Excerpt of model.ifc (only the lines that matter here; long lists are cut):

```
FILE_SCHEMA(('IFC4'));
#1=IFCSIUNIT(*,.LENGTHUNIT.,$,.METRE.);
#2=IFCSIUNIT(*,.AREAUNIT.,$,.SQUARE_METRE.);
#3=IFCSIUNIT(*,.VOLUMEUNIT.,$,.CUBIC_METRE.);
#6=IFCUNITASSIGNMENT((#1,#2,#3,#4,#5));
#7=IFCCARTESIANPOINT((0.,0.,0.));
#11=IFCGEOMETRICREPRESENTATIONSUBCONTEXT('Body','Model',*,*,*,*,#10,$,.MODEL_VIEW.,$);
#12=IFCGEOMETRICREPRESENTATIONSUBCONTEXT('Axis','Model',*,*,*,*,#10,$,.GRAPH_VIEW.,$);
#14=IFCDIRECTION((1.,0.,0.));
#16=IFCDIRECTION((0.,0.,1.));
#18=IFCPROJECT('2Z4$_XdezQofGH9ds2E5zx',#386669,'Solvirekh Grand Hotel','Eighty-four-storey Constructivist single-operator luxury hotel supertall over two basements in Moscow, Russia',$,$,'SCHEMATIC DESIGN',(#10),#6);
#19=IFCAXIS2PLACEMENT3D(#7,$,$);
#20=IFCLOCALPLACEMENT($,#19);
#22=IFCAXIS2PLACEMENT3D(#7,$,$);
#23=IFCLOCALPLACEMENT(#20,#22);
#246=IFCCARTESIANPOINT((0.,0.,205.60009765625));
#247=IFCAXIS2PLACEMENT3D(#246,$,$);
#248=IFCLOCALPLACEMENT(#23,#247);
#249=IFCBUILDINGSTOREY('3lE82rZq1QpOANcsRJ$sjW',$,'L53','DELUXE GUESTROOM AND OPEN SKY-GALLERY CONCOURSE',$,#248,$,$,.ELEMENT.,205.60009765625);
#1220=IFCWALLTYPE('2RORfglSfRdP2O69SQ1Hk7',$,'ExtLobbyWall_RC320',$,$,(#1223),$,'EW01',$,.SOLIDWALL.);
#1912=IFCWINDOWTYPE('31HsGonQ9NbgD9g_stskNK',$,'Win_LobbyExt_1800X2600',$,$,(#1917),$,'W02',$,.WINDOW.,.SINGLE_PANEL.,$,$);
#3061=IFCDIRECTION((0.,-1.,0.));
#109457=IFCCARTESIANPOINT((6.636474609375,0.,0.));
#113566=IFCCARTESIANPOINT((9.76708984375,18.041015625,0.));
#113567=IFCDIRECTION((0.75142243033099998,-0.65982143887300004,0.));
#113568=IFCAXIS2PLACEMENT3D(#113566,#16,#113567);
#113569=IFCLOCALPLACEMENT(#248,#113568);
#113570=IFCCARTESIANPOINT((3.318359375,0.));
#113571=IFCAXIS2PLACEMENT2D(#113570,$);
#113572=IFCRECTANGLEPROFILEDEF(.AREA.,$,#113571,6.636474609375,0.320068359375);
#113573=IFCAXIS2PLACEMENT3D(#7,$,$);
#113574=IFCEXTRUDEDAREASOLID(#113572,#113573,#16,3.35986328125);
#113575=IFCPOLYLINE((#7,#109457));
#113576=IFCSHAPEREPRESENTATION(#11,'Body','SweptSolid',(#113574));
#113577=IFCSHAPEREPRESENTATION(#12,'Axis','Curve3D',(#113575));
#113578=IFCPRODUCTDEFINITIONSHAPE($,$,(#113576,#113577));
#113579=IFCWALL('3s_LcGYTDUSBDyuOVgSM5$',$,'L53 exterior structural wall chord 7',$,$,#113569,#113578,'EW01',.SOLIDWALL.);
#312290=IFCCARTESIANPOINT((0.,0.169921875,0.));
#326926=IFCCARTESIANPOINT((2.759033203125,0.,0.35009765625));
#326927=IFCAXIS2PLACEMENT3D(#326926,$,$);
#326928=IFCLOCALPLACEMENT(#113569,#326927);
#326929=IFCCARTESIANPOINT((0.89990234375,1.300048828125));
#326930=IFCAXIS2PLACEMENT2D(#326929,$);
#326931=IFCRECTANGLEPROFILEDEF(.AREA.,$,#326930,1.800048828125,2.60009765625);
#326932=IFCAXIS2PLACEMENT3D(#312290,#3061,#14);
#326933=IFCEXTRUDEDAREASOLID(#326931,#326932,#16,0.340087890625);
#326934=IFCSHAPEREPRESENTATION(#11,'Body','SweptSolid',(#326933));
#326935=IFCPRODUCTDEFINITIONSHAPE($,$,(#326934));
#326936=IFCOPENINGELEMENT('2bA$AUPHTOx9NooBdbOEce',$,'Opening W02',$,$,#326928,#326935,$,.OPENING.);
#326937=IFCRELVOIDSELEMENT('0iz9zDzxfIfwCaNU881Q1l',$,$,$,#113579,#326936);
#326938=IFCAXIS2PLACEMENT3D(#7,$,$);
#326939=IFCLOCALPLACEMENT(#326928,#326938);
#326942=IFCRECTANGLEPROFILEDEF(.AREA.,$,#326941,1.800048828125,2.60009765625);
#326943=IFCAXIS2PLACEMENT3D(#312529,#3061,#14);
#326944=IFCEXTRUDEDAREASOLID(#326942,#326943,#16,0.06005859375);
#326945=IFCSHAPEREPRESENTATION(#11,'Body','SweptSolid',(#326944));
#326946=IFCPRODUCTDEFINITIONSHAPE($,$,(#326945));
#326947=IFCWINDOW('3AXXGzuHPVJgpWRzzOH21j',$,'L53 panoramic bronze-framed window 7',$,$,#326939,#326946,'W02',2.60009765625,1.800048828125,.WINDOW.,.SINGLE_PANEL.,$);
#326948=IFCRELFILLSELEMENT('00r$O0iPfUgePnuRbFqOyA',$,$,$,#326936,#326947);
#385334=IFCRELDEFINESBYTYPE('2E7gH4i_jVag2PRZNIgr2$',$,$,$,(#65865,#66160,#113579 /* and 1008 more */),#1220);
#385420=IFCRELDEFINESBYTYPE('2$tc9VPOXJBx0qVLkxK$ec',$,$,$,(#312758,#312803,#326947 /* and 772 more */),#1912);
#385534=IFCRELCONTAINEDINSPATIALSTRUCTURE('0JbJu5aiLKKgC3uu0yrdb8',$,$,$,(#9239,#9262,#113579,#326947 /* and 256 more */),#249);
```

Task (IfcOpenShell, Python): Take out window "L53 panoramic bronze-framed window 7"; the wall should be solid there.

```python
import ifcopenshell
import ifcopenshell.api.feature
import ifcopenshell.api.root
import ifcopenshell.geom
import ifcopenshell.util.shape

model = ifcopenshell.open("model.ifc")
settings = ifcopenshell.geom.settings()


def volume(element):
    """Net volume in cubic metres, openings subtracted."""
    shape = ifcopenshell.geom.create_shape(settings, element)
    return ifcopenshell.util.shape.get_volume(shape.geometry)


window = model.by_guid("3AXXGzuHPVJgpWRzzOH21j")
opening = window.FillsVoids[0].RelatingOpeningElement
wall = opening.VoidsElements[0].RelatingBuildingElement
before = volume(wall)

ifcopenshell.api.root.remove_product(model, product=window)
ifcopenshell.api.feature.remove_feature(model, feature=opening)

after = volume(wall)

print(f"wall volume {before:.3f} -> {after:.3f} m3")

model.write("model_v2.ifc")
```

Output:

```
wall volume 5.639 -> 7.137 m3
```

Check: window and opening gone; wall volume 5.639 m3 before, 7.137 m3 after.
